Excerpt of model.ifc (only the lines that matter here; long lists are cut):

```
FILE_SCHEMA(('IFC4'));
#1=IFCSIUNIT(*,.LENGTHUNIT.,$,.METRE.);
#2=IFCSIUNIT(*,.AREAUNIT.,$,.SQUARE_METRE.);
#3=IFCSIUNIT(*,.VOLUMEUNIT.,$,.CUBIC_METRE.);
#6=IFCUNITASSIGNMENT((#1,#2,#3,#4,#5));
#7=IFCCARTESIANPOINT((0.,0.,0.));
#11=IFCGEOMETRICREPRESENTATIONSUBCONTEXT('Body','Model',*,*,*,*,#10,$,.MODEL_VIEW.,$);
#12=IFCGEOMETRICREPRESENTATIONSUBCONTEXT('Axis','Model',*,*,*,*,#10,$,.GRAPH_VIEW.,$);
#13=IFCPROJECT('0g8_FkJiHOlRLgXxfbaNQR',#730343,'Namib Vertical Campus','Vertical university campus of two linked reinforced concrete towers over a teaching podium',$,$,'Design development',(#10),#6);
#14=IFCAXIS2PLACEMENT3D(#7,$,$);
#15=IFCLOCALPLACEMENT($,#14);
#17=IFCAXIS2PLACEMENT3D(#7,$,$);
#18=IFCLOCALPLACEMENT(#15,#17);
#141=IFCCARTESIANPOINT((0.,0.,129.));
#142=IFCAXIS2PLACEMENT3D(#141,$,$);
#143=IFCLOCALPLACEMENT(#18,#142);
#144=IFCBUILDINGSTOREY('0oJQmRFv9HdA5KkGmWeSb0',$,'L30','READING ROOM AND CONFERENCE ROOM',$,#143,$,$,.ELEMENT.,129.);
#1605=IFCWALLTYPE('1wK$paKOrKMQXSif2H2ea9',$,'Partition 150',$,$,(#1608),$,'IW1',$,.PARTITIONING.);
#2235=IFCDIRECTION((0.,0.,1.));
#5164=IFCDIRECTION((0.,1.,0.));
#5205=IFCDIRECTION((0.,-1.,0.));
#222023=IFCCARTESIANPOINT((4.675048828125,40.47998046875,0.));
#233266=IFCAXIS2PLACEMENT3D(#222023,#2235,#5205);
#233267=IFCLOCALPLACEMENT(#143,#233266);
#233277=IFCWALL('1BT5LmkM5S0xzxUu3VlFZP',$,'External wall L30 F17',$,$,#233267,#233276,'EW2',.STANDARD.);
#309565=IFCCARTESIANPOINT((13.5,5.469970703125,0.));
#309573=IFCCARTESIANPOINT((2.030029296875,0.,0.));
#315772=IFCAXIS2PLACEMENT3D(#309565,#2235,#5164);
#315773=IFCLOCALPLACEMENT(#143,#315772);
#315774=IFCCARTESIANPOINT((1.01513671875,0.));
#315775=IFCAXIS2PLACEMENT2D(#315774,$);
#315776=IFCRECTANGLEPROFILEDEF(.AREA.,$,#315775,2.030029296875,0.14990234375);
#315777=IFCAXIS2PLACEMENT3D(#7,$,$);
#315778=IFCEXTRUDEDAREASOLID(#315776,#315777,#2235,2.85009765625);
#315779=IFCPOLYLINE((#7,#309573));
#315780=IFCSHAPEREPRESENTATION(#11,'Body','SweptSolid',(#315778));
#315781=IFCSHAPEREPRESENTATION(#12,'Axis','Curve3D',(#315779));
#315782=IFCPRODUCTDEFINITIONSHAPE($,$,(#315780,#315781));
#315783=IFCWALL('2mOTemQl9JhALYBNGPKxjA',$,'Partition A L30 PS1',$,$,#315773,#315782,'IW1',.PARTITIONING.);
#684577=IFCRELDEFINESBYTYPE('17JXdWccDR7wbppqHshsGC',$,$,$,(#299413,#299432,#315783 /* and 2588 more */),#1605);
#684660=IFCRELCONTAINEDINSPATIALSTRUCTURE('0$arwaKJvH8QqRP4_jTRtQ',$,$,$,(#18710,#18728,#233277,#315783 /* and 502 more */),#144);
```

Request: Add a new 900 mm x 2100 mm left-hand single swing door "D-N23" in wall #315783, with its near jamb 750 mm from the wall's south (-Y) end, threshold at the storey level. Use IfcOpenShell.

```python
import numpy as np
import ifcopenshell
import ifcopenshell.api.feature
import ifcopenshell.api.geometry
import ifcopenshell.api.root
import ifcopenshell.api.spatial
import ifcopenshell.geom
import ifcopenshell.util.element
import ifcopenshell.util.placement
import ifcopenshell.util.representation
import ifcopenshell.util.shape
import ifcopenshell.util.unit

model = ifcopenshell.open("model.ifc")
unit_scale = ifcopenshell.util.unit.calculate_unit_scale(model)
settings = ifcopenshell.geom.settings()


def volume(element):
    """Net volume in cubic metres, openings subtracted."""
    shape = ifcopenshell.geom.create_shape(settings, element)
    return ifcopenshell.util.shape.get_volume(shape.geometry)


wall = model.by_guid("2mOTemQl9JhALYBNGPKxjA")
storey = ifcopenshell.util.element.get_container(wall, ifc_class="IfcBuildingStorey")
context = ifcopenshell.util.representation.get_context(model, "Model", "Body", "MODEL_VIEW")
before = volume(wall)

width, height, from_end, sill = 0.9, 2.1, 0.75, 0.0  # metres

# The wall runs along its own X axis, and the end named is its -X end.
wall_shape = ifcopenshell.geom.create_shape(settings, wall)
x, y, z = ifcopenshell.util.shape.get_vertices(wall_shape.geometry).T
start = x.min() + from_end
face, thickness = float(y.min()), float(y.max() - y.min())
wall_matrix = ifcopenshell.util.placement.get_local_placement(wall.ObjectPlacement)
level = ifcopenshell.util.placement.get_local_placement(storey.ObjectPlacement)[2, 3]


def in_wall(x, y):
    """Placement at x, y metres in the wall's axes, at sill height."""
    matrix = wall_matrix.copy()
    matrix[:, 3] = wall_matrix @ np.array([x / unit_scale, y / unit_scale, 0.0, 1.0])
    matrix[2, 3] = level + sill / unit_scale
    return matrix


# Opening: a box that overshoots both wall faces by 50 mm.
opening = ifcopenshell.api.root.create_entity(model, ifc_class="IfcOpeningElement", predefined_type="OPENING")
box = ifcopenshell.api.geometry.add_wall_representation(
    model, context=context, length=width, height=height, thickness=thickness + 0.1
)
ifcopenshell.api.geometry.assign_representation(model, product=opening, representation=box)
ifcopenshell.api.geometry.edit_object_placement(model, product=opening, matrix=in_wall(start, face - 0.05), is_si=False)
ifcopenshell.api.feature.add_feature(model, feature=opening, element=wall)

door = ifcopenshell.api.root.create_entity(model, ifc_class="IfcDoor", name="D-N23", predefined_type="DOOR")
door.OverallWidth, door.OverallHeight = width / unit_scale, height / unit_scale
door.OperationType = "SINGLE_SWING_LEFT"
body = ifcopenshell.api.geometry.add_door_representation(
    model,
    context=context,
    overall_width=door.OverallWidth,
    overall_height=door.OverallHeight,
    operation_type="SINGLE_SWING_LEFT",
    lining_properties={"LiningDepth": thickness / unit_scale, "ThresholdDepth": thickness / unit_scale},
)
ifcopenshell.api.geometry.assign_representation(model, product=door, representation=body)
ifcopenshell.api.spatial.assign_container(model, products=[door], relating_structure=storey)
ifcopenshell.api.feature.add_filling(model, opening=opening, element=door)

# The lining spans the wall, so the door starts at the wall face.
ifcopenshell.api.geometry.edit_object_placement(model, product=door, matrix=in_wall(start, face), is_si=False)

after = volume(wall)

print(f"wall volume {before:.3f} -> {after:.3f} m3")

model.write("model_v2.ifc")
```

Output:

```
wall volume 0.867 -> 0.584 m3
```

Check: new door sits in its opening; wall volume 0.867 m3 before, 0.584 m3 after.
